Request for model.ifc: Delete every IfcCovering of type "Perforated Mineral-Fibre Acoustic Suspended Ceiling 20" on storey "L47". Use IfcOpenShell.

First a look at what the model holds.

```python
import ifcopenshell
import ifcopenshell.util.element

model = ifcopenshell.open("model.ifc")
print(model.schema)
storey = next(s for s in model.by_type("IfcBuildingStorey") if s.Name == "L47")
coverings = [e for e in ifcopenshell.util.element.get_decomposition(storey) if e.is_a("IfcCovering")]
seen = {}
for e in coverings:
    element_type = ifcopenshell.util.element.get_type(e)
    name = element_type.Name if element_type not in (None, e) else None
    seen[name] = seen.get(name, 0) + 1
for name, count in sorted(seen.items(), key=str):
    print(count, "x", name)
```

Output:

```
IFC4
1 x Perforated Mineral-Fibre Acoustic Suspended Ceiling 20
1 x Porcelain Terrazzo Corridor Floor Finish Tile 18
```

```python
import ifcopenshell
import ifcopenshell.api.root
import ifcopenshell.util.element

model = ifcopenshell.open("model.ifc")

storey = next(s for s in model.by_type("IfcBuildingStorey") if s.Name == "L47")
coverings = [e for e in ifcopenshell.util.element.get_decomposition(storey) if e.is_a("IfcCovering")]
targets = [e for e in coverings if (t := ifcopenshell.util.element.get_type(e)) not in (None, e) and t.Name == "Perforated Mineral-Fibre Acoustic Suspended Ceiling 20"]

for e in targets:
    ifcopenshell.api.root.remove_product(model, product=e)
print(len(targets), "removed")

model.write("model_updated.ifc")
```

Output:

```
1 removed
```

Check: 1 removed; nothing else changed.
